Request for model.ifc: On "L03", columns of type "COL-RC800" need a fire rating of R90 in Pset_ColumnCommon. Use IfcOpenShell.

First a look at what the model holds.

```python
import ifcopenshell
import ifcopenshell.util.element

model = ifcopenshell.open("model.ifc")
print(model.schema)
storey = next(s for s in model.by_type("IfcBuildingStorey") if s.Name == "L03")
columns = [e for e in ifcopenshell.util.element.get_decomposition(storey) if e.is_a("IfcColumn")]
seen = {}
for e in columns:
    element_type = ifcopenshell.util.element.get_type(e)
    key = (element_type.Name if element_type != e and element_type else None, ifcopenshell.util.element.get_pset(e, "Pset_ColumnCommon", "FireRating"))
    seen[key] = seen.get(key, 0) + 1
for (name, value), count in sorted(seen.items(), key=str):
    print(count, "x", name, "|", value)
```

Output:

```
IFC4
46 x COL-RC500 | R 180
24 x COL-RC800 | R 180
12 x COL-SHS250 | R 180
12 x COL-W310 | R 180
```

```python
import ifcopenshell
import ifcopenshell.api.pset
import ifcopenshell.util.element

model = ifcopenshell.open("model.ifc")

storey = next(s for s in model.by_type("IfcBuildingStorey") if s.Name == "L03")
columns = [e for e in ifcopenshell.util.element.get_decomposition(storey) if e.is_a("IfcColumn")]

count = 0
for e in columns:
    element_type = ifcopenshell.util.element.get_type(e)
    if element_type in (None, e) or element_type.Name != "COL-RC800":
        continue
    # add_pset returns the element's existing set when there is one.
    pset = ifcopenshell.api.pset.add_pset(model, product=e, name="Pset_ColumnCommon")
    ifcopenshell.api.pset.edit_pset(model, pset=pset, properties={"FireRating": "R90"})
    count += 1

print(count, "columns updated")

model.write("model_edited.ifc")
```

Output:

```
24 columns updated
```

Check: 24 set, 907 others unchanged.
